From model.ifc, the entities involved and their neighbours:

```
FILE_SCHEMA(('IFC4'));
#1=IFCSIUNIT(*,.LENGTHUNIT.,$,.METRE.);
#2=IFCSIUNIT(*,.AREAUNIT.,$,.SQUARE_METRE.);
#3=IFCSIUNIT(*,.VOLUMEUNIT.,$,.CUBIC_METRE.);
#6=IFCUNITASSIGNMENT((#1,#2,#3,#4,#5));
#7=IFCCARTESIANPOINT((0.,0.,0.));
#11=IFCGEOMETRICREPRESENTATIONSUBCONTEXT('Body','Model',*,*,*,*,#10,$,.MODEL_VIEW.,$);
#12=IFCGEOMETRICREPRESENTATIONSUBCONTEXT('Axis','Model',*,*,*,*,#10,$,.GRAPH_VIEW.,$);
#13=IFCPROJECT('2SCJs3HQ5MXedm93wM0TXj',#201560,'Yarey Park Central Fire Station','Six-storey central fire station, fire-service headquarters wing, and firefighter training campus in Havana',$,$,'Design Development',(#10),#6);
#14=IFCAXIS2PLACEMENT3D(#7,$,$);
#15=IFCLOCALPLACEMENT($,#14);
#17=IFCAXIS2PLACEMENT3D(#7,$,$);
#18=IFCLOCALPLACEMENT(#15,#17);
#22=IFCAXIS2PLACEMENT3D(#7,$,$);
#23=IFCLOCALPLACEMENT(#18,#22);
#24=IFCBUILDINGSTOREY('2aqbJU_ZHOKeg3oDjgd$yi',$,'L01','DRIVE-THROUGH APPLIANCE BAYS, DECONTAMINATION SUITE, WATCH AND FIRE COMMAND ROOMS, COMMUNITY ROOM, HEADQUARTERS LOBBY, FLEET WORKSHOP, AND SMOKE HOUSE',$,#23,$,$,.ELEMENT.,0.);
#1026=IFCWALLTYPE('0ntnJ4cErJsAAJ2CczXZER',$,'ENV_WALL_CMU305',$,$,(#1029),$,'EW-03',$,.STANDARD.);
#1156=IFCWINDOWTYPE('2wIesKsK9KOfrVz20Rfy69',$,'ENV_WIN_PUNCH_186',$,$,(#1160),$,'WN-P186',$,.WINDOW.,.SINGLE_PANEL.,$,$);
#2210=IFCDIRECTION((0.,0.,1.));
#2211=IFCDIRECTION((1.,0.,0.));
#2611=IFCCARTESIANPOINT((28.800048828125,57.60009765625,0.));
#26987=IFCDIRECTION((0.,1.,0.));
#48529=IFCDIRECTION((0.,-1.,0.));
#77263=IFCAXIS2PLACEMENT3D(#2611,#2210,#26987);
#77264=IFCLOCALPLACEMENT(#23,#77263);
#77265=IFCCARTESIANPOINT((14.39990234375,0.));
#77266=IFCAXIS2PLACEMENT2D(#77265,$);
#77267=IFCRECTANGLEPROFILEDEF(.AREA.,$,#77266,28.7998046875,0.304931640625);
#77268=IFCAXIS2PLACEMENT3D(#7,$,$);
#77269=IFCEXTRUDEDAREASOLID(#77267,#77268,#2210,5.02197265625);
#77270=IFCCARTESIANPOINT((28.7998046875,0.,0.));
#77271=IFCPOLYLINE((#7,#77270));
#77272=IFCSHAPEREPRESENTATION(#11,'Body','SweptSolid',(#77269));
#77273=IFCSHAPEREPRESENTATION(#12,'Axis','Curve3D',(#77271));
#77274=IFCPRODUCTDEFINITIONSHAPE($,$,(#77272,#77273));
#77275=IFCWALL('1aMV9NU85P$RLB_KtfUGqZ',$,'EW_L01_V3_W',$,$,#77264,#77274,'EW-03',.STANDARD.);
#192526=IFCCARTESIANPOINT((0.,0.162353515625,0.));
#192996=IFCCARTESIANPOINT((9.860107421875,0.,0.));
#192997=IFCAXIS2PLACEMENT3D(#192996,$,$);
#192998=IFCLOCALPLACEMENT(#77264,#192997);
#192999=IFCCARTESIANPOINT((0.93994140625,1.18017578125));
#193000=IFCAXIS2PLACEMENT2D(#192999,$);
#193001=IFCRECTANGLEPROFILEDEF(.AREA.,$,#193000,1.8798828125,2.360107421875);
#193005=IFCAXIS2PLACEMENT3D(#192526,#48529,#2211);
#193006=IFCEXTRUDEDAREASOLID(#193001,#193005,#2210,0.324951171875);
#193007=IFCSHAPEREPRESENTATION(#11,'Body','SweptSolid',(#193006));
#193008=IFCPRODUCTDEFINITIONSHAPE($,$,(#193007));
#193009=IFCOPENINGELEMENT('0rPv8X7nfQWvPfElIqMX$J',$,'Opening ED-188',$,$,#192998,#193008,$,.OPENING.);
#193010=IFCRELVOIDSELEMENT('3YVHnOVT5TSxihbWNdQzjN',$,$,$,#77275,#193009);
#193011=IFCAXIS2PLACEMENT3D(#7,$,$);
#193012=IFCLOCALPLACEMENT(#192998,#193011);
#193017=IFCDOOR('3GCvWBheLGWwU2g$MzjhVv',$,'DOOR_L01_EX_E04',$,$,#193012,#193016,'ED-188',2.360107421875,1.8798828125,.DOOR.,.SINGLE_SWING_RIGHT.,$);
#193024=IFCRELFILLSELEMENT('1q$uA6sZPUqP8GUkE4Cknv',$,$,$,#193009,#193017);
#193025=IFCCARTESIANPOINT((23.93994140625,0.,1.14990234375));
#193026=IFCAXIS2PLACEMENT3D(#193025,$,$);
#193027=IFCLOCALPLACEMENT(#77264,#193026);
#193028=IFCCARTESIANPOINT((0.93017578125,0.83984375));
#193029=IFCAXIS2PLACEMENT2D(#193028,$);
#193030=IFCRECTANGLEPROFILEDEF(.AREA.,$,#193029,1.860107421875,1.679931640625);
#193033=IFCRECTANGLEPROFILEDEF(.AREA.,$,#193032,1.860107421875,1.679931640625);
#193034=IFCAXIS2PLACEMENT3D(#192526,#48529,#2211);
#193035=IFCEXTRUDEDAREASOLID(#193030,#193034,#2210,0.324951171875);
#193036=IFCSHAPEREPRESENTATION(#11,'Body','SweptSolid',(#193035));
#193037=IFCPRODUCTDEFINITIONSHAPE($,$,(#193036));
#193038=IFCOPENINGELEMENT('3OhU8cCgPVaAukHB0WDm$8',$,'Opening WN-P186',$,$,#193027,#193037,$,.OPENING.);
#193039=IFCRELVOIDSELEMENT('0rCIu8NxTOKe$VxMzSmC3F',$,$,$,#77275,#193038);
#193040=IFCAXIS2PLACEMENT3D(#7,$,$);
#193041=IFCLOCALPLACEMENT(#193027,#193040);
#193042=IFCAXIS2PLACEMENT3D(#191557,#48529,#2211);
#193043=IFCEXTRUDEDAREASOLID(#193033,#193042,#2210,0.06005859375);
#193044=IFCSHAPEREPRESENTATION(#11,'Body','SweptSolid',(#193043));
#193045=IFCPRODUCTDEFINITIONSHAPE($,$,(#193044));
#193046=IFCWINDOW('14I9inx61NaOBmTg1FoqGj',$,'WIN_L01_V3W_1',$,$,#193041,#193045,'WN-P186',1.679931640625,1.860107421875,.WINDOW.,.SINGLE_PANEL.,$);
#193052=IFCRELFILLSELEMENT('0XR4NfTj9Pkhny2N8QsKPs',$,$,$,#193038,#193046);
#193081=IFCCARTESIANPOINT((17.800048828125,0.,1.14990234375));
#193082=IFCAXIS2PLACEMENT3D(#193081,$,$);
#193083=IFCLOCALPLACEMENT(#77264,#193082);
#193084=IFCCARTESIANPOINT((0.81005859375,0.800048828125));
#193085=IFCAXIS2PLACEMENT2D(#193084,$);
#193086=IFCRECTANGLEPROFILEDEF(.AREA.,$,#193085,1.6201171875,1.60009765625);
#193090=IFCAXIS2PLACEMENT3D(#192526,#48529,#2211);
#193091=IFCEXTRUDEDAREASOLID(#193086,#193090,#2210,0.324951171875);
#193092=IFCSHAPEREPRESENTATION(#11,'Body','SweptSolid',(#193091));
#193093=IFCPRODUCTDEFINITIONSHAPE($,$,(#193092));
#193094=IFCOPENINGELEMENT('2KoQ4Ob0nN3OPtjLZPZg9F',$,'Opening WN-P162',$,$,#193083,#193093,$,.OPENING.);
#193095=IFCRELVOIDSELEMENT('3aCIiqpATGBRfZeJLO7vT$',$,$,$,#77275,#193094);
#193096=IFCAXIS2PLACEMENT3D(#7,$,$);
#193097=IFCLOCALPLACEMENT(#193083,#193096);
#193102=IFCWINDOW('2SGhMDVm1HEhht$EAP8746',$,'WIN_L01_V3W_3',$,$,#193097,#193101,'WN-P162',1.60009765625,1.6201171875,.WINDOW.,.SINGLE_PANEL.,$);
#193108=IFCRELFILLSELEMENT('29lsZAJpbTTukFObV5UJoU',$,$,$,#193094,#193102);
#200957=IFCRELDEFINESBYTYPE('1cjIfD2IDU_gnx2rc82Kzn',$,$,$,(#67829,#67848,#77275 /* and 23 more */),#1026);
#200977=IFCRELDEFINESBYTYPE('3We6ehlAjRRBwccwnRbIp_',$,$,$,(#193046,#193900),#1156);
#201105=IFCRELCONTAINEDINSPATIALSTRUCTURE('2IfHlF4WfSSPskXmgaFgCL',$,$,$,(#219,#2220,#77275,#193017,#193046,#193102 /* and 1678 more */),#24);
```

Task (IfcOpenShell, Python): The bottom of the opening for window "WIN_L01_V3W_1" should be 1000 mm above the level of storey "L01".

```python
import numpy as np
import ifcopenshell
import ifcopenshell.api.geometry
import ifcopenshell.geom
import ifcopenshell.util.element
import ifcopenshell.util.placement
import ifcopenshell.util.shape
import ifcopenshell.util.unit

model = ifcopenshell.open("model.ifc")
unit_scale = ifcopenshell.util.unit.calculate_unit_scale(model)

window = model.by_id(193046)
opening = window.FillsVoids[0].RelatingOpeningElement
storey = ifcopenshell.util.element.get_container(window, ifc_class="IfcBuildingStorey")
level = ifcopenshell.util.placement.get_local_placement(storey.ObjectPlacement)[2, 3]

# The opening's origin need not be at the sill, so measure its lowest point.
shape = ifcopenshell.geom.create_shape(ifcopenshell.geom.settings(), opening)
bottom = ifcopenshell.util.shape.get_shape_bottom_elevation(shape, shape.geometry) / unit_scale
dz = level + 1.0 - bottom

shift = np.array([0.0, 0.0, dz])
# The window is placed relative to its opening, so it follows when the opening moves.
matrix = ifcopenshell.util.placement.get_local_placement(opening.ObjectPlacement)
matrix[:3, 3] += shift
ifcopenshell.api.geometry.edit_object_placement(
    model, product=opening, matrix=matrix, is_si=False, should_transform_children=True
)

print(f"moved by {dz * unit_scale:+.3f} m")

model.write("model_updated.ifc")
```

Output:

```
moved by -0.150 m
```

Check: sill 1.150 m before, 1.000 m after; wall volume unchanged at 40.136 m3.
